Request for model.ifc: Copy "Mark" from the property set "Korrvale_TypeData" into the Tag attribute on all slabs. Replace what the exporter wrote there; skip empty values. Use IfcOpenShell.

First a look at what the model holds.

```python
import ifcopenshell
import ifcopenshell.util.element

model = ifcopenshell.open("model.ifc")
print(model.schema)
slabs = model.by_type("IfcSlab")
print(len(slabs), "slabs")
for e in slabs[:8]:
    source = ifcopenshell.util.element.get_pset(e, "Korrvale_TypeData", "Mark")
    target = e.Tag
    print(e.id(), repr(source), repr(target), sep=" | ")
```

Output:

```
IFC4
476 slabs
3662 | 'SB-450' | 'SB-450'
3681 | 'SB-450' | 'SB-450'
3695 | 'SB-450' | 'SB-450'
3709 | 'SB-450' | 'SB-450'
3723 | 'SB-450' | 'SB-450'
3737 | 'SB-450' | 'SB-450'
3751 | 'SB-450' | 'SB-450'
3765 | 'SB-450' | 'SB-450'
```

```python
import ifcopenshell
import ifcopenshell.util.element

model = ifcopenshell.open("model.ifc")

count = 0
for e in model.by_type("IfcSlab"):
    value = ifcopenshell.util.element.get_pset(e, "Korrvale_TypeData", "Mark")
    current = e.Tag
    if not value or not value.strip() or current == value:
        continue
    e.Tag = value
    count += 1

print(count, "slabs updated")

model.write("model_rev.ifc")
```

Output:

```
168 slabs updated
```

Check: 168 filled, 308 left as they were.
